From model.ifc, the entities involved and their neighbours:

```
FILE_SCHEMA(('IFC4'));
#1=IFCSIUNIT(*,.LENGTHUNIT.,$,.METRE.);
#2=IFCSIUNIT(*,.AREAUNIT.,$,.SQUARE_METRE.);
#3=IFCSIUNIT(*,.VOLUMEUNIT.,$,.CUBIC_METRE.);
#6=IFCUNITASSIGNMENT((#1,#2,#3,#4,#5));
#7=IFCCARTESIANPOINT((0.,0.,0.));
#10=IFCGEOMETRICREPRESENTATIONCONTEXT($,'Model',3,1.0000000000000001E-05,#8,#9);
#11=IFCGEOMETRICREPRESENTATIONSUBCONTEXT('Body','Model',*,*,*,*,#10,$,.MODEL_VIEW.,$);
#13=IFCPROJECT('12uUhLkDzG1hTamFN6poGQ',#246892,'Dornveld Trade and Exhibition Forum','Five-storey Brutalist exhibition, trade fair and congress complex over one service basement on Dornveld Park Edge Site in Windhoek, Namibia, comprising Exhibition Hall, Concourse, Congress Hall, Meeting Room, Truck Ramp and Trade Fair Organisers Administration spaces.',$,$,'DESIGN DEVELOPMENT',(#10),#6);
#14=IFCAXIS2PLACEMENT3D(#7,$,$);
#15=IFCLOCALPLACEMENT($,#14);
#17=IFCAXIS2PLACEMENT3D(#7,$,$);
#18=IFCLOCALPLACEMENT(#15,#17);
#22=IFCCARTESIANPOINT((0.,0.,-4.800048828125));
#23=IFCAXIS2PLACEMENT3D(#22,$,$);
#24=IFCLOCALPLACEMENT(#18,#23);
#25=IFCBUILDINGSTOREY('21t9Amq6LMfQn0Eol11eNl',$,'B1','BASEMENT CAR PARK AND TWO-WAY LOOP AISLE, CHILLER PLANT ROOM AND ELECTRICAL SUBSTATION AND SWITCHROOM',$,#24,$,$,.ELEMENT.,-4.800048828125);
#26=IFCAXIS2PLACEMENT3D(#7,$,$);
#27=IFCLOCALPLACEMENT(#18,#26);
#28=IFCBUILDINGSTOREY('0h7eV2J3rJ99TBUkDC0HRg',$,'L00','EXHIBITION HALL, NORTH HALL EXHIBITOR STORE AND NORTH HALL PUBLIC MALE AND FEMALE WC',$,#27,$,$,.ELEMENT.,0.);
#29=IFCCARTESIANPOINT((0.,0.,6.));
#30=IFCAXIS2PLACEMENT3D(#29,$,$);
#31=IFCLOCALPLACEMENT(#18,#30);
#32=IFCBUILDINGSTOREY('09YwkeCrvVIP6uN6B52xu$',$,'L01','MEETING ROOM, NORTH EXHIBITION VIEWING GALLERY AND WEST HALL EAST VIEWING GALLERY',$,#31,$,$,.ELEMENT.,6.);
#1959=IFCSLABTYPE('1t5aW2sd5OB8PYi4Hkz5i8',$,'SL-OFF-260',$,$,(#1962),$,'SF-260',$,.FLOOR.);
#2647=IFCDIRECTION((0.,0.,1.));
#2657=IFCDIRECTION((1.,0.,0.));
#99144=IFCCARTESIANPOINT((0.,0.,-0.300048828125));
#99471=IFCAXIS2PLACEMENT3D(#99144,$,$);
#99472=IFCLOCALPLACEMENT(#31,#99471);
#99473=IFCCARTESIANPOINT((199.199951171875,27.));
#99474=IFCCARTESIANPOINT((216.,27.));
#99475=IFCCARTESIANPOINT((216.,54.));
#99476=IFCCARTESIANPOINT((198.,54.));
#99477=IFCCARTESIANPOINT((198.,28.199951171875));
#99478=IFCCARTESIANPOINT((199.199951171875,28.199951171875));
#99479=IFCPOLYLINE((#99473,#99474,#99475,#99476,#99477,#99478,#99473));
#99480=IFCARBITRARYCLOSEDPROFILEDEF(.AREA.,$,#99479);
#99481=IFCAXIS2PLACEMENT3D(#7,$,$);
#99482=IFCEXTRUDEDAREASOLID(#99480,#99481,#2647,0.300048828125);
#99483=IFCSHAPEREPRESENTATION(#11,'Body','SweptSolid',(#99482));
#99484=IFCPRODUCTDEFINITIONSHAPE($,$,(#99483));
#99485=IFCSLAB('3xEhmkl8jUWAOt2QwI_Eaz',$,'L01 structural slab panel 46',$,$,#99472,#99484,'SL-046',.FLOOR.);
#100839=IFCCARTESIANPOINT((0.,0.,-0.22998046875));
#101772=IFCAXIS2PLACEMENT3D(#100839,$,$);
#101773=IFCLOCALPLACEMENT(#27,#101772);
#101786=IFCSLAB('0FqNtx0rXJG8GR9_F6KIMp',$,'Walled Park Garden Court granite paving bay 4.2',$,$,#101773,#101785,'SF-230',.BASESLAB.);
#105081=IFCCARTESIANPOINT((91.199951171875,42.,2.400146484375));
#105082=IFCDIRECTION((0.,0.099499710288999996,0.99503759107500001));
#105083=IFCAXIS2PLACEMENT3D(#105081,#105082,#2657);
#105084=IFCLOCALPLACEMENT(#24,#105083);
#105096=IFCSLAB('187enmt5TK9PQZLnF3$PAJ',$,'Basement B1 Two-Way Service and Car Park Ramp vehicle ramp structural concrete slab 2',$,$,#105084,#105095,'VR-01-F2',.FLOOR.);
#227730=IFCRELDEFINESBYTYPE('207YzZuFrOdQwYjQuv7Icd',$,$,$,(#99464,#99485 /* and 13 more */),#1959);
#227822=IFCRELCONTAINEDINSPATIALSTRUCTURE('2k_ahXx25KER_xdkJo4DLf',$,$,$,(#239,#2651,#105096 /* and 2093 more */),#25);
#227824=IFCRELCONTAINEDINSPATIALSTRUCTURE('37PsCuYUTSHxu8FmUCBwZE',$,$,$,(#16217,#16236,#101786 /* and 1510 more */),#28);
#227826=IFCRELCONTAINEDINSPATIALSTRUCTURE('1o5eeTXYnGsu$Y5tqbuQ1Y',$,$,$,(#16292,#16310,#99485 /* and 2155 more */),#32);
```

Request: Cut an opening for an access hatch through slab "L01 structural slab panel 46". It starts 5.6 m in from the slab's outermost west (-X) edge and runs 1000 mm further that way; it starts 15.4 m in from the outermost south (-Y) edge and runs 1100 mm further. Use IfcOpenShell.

```python
import numpy as np
import ifcopenshell
import ifcopenshell.api.feature
import ifcopenshell.api.geometry
import ifcopenshell.api.root
import ifcopenshell.geom
import ifcopenshell.util.placement
import ifcopenshell.util.representation
import ifcopenshell.util.shape
import ifcopenshell.util.unit

model = ifcopenshell.open("model.ifc")
unit_scale = ifcopenshell.util.unit.calculate_unit_scale(model)
settings = ifcopenshell.geom.settings()


def volume(element):
    """Net volume in cubic metres, openings subtracted."""
    shape = ifcopenshell.geom.create_shape(settings, element)
    return ifcopenshell.util.shape.get_volume(shape.geometry)


slab = model.by_guid("3xEhmkl8jUWAOt2QwI_Eaz")
before = volume(slab)

# Extent in the slab's own axes, in metres. The edges named are its -X and -Y sides.
slab_shape = ifcopenshell.geom.create_shape(settings, slab)
vertices = ifcopenshell.util.shape.get_vertices(slab_shape.geometry)
x_min, y_min, bottom = vertices.min(axis=0)
top = vertices[:, 2].max()

opening = ifcopenshell.api.root.create_entity(model, ifc_class="IfcOpeningElement", name="Access hatch opening", predefined_type="OPENING")
context = ifcopenshell.util.representation.get_context(model, "Model", "Body", "MODEL_VIEW")
width, depth = 1, 1.1
outline = [(0.0, 0.0), (width, 0.0), (width, depth), (0.0, depth), (0.0, 0.0)]
# Overshoot both faces by 50 mm so the cut is clean.
shape = ifcopenshell.api.geometry.add_slab_representation(
    model, context=context, depth=top - bottom + 0.1, polyline=outline
)
ifcopenshell.api.geometry.assign_representation(model, product=opening, representation=shape)

matrix = ifcopenshell.util.placement.get_local_placement(slab.ObjectPlacement)
matrix[:, 3] = matrix @ np.append(np.array([x_min + 5.6, y_min + 15.4, bottom - 0.05]) / unit_scale, 1.0)
ifcopenshell.api.geometry.edit_object_placement(model, product=opening, matrix=matrix, is_si=False)
ifcopenshell.api.feature.add_feature(model, feature=opening, element=slab)

after = volume(slab)

print(f"slab volume {before:.3f} -> {after:.3f} m3")

model.write("model-out.ifc")
```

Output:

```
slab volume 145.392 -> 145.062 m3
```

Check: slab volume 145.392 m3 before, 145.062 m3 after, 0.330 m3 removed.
